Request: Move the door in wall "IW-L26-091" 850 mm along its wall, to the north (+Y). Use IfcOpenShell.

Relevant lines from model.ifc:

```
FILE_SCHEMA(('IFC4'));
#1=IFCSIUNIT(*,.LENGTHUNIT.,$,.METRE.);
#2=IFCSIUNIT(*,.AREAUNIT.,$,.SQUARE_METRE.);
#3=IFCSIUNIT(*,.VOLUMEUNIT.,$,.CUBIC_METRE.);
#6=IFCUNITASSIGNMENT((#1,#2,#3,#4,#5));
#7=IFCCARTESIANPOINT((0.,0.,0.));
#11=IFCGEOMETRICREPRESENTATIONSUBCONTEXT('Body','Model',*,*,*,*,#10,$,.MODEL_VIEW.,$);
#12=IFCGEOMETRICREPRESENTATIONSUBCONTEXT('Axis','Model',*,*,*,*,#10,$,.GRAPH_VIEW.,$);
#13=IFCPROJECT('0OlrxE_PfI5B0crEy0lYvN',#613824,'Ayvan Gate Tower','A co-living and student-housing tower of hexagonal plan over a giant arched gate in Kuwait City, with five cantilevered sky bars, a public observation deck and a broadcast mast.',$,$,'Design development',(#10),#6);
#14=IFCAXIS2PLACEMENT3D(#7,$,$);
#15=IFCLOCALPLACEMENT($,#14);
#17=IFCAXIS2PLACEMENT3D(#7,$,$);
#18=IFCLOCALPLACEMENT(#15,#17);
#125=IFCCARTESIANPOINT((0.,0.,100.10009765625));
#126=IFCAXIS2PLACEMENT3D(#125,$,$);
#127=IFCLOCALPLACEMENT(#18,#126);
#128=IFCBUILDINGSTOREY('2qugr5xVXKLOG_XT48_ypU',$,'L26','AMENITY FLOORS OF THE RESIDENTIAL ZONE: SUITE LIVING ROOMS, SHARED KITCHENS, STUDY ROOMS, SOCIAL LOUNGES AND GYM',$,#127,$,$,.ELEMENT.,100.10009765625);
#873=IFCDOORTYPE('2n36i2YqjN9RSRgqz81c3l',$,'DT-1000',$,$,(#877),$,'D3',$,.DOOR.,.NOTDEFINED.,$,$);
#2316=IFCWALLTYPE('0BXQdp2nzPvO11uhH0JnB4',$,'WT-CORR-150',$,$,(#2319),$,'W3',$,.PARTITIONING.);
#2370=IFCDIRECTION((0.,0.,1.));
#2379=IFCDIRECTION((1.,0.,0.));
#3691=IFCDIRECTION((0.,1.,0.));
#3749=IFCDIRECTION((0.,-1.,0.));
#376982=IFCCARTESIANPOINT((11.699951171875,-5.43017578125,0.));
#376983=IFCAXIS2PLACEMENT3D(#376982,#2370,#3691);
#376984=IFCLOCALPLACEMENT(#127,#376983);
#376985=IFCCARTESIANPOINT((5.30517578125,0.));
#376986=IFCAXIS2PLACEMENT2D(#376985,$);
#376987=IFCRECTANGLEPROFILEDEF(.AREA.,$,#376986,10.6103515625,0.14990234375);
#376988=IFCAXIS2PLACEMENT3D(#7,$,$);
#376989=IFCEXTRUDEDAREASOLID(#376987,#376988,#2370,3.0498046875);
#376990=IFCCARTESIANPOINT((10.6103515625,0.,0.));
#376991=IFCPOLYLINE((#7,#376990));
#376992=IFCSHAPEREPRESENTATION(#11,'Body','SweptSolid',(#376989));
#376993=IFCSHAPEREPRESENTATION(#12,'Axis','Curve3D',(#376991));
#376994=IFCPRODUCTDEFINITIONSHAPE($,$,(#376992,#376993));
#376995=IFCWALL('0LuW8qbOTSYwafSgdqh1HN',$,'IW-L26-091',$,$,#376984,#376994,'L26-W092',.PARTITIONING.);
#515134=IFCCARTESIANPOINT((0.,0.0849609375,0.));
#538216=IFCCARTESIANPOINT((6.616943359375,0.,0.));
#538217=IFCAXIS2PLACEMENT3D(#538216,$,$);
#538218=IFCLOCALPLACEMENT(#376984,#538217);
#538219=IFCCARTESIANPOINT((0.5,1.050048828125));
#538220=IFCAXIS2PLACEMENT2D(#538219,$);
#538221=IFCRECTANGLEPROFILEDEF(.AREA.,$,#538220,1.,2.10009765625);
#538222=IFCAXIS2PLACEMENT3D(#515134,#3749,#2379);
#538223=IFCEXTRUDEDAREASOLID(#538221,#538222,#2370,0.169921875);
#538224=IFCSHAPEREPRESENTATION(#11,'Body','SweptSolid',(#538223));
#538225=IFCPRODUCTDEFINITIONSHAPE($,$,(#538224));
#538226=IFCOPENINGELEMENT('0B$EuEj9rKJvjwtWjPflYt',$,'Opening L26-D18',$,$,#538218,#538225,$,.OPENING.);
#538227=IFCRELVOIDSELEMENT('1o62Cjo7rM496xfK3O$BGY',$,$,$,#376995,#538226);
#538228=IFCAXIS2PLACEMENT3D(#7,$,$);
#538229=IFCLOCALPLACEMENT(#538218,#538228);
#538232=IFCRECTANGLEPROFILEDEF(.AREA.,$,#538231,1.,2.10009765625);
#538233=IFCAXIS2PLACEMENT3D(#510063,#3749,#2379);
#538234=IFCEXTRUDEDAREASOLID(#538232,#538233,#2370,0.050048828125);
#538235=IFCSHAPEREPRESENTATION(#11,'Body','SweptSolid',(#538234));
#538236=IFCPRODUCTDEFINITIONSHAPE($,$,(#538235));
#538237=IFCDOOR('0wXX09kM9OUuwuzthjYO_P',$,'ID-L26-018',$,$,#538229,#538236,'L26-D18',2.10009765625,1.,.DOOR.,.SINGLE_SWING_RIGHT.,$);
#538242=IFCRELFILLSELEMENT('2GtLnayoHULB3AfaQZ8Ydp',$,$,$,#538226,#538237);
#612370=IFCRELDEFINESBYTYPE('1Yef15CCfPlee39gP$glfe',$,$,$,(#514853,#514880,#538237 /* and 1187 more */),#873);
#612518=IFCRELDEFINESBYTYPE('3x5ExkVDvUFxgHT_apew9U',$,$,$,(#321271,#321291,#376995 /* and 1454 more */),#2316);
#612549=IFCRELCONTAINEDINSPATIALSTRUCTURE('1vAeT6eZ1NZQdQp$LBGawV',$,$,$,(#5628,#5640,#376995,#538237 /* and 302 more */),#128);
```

```python
import ifcopenshell
import ifcopenshell.api.geometry
import ifcopenshell.util.placement
import ifcopenshell.util.unit

model = ifcopenshell.open("model.ifc")
unit_scale = ifcopenshell.util.unit.calculate_unit_scale(model)

door = model.by_guid("0wXX09kM9OUuwuzthjYO_P")
opening = door.FillsVoids[0].RelatingOpeningElement
wall = opening.VoidsElements[0].RelatingBuildingElement

wall_matrix = ifcopenshell.util.placement.get_local_placement(wall.ObjectPlacement)
shift = wall_matrix[:3, 0] * 0.85 / unit_scale
before = ifcopenshell.util.placement.get_local_placement(door.ObjectPlacement)[:3, 3].copy()

# The door is placed relative to its opening, so it follows when the opening moves.
matrix = ifcopenshell.util.placement.get_local_placement(opening.ObjectPlacement)
matrix[:3, 3] += shift
ifcopenshell.api.geometry.edit_object_placement(
    model, product=opening, matrix=matrix, is_si=False, should_transform_children=True
)

after = ifcopenshell.util.placement.get_local_placement(door.ObjectPlacement)[:3, 3]
print("door moved by", (after - before).round(3) + 0.0)

model.write("model_rev.ifc")
```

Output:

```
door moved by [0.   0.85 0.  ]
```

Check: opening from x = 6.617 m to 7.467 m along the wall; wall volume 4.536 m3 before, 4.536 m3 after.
